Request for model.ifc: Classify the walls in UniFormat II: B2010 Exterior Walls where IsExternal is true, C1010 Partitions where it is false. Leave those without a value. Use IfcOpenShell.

First a look at what the model holds.

```python
import ifcopenshell
import ifcopenshell.util.element

model = ifcopenshell.open("model.ifc")
print(model.schema)
print("classifications:", [c.Name for c in model.by_type("IfcClassification")])
values = [ifcopenshell.util.element.get_pset(e, "Pset_WallCommon", "IsExternal") for e in model.by_type("IfcWall")]
for value in (True, False, None):
    print("IsExternal", value, values.count(value))
```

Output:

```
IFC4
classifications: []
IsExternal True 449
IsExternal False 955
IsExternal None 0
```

```python
import ifcopenshell
import ifcopenshell.api.classification
import ifcopenshell.util.element

model = ifcopenshell.open("model.ifc")

system = ifcopenshell.api.classification.add_classification(model, classification="UniFormat II")

walls = model.by_type("IfcWall")
external = {e: ifcopenshell.util.element.get_pset(e, "Pset_WallCommon", "IsExternal") for e in walls}
for flag, code, name in ((True, "B2010", "Exterior Walls"), (False, "C1010", "Partitions")):
    products = [e for e in walls if external[e] is flag]
    ifcopenshell.api.classification.add_reference(
        model, products=products, classification=system, identification=code, name=name
    )
    print(code, len(products))

model.write("model-out.ifc")
```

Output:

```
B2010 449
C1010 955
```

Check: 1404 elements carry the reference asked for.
